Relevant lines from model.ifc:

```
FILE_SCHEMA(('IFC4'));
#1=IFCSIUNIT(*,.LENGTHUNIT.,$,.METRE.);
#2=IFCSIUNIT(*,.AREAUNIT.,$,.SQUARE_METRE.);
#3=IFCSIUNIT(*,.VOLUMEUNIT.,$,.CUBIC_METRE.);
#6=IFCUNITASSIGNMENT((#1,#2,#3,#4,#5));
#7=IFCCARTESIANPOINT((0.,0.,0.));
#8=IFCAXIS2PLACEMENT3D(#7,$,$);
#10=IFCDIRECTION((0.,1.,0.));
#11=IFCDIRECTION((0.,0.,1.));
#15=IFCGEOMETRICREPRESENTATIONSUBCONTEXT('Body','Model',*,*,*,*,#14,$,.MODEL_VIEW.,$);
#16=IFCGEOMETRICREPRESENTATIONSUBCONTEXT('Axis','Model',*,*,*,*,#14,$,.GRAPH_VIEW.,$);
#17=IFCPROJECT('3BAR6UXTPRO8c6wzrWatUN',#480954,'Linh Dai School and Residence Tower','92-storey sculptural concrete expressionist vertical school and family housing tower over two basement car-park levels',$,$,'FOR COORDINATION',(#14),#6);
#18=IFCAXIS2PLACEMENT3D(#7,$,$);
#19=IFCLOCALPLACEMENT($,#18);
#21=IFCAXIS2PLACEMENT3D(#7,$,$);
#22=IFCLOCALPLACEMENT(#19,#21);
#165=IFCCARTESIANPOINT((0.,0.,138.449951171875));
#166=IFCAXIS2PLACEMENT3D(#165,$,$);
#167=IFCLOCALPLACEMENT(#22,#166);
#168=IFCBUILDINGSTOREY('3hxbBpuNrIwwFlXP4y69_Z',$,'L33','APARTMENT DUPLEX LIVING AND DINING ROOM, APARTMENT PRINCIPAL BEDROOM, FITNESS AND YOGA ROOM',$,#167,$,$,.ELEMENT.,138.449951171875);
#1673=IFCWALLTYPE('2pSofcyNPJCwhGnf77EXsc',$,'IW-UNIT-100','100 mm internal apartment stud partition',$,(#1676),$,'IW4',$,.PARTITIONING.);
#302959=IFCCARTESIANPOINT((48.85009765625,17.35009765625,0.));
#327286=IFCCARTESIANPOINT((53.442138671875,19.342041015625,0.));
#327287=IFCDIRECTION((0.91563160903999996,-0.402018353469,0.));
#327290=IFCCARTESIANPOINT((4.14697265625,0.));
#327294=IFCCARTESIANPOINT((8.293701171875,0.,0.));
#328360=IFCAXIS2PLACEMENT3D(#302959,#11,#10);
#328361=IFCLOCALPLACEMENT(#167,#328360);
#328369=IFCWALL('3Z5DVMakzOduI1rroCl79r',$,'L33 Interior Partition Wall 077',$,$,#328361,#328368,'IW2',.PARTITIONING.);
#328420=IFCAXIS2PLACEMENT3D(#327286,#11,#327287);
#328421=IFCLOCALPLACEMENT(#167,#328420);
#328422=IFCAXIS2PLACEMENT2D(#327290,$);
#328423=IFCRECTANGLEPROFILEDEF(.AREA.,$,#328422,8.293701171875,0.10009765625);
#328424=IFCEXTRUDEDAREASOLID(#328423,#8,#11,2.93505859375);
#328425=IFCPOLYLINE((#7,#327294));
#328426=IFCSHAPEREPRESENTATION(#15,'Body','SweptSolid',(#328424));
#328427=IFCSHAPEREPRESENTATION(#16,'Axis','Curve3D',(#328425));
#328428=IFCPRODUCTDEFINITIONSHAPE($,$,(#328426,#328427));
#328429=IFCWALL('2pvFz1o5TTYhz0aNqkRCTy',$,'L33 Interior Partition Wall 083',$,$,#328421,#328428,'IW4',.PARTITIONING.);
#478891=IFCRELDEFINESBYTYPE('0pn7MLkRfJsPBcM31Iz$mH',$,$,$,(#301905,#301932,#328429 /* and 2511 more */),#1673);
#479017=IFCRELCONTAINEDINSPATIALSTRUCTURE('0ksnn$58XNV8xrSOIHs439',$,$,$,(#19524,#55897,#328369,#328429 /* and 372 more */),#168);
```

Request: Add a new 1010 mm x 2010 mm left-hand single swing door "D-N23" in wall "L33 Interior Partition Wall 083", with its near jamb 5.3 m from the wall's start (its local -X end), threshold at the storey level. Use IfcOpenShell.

```python
import numpy as np
import ifcopenshell
import ifcopenshell.api.feature
import ifcopenshell.api.geometry
import ifcopenshell.api.root
import ifcopenshell.api.spatial
import ifcopenshell.geom
import ifcopenshell.util.element
import ifcopenshell.util.placement
import ifcopenshell.util.representation
import ifcopenshell.util.shape
import ifcopenshell.util.unit

model = ifcopenshell.open("model.ifc")
unit_scale = ifcopenshell.util.unit.calculate_unit_scale(model)
settings = ifcopenshell.geom.settings()


def volume(element):
    """Net volume in cubic metres, openings subtracted."""
    shape = ifcopenshell.geom.create_shape(settings, element)
    return ifcopenshell.util.shape.get_volume(shape.geometry)


wall = model.by_guid("2pvFz1o5TTYhz0aNqkRCTy")
storey = ifcopenshell.util.element.get_container(wall, ifc_class="IfcBuildingStorey")
context = ifcopenshell.util.representation.get_context(model, "Model", "Body", "MODEL_VIEW")
before = volume(wall)

width, height, from_end, sill = 1.01, 2.01, 5.3, 0.0  # metres

# The wall runs along its own X axis, and the end named is its -X end.
wall_shape = ifcopenshell.geom.create_shape(settings, wall)
x, y, z = ifcopenshell.util.shape.get_vertices(wall_shape.geometry).T
start = x.min() + from_end
face, thickness = float(y.min()), float(y.max() - y.min())
wall_matrix = ifcopenshell.util.placement.get_local_placement(wall.ObjectPlacement)
level = ifcopenshell.util.placement.get_local_placement(storey.ObjectPlacement)[2, 3]


def in_wall(x, y):
    """Placement at x, y metres in the wall's axes, at sill height."""
    matrix = wall_matrix.copy()
    matrix[:, 3] = wall_matrix @ np.array([x / unit_scale, y / unit_scale, 0.0, 1.0])
    matrix[2, 3] = level + sill / unit_scale
    return matrix


# Opening: a box that overshoots both wall faces by 50 mm.
opening = ifcopenshell.api.root.create_entity(model, ifc_class="IfcOpeningElement", predefined_type="OPENING")
box = ifcopenshell.api.geometry.add_wall_representation(
    model, context=context, length=width, height=height, thickness=thickness + 0.1
)
ifcopenshell.api.geometry.assign_representation(model, product=opening, representation=box)
ifcopenshell.api.geometry.edit_object_placement(model, product=opening, matrix=in_wall(start, face - 0.05), is_si=False)
ifcopenshell.api.feature.add_feature(model, feature=opening, element=wall)

door = ifcopenshell.api.root.create_entity(model, ifc_class="IfcDoor", name="D-N23", predefined_type="DOOR")
door.OverallWidth, door.OverallHeight = width / unit_scale, height / unit_scale
door.OperationType = "SINGLE_SWING_LEFT"
body = ifcopenshell.api.geometry.add_door_representation(
    model,
    context=context,
    overall_width=door.OverallWidth,
    overall_height=door.OverallHeight,
    operation_type="SINGLE_SWING_LEFT",
    lining_properties={"LiningDepth": thickness / unit_scale, "ThresholdDepth": thickness / unit_scale},
)
ifcopenshell.api.geometry.assign_representation(model, product=door, representation=body)
ifcopenshell.api.spatial.assign_container(model, products=[door], relating_structure=storey)
ifcopenshell.api.feature.add_filling(model, opening=opening, element=door)

# The lining spans the wall, so the door starts at the wall face.
ifcopenshell.api.geometry.edit_object_placement(model, product=door, matrix=in_wall(start, face), is_si=False)

after = volume(wall)

print(f"wall volume {before:.3f} -> {after:.3f} m3")

model.write("model_v2.ifc")
```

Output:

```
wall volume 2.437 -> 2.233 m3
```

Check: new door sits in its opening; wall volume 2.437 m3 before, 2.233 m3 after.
